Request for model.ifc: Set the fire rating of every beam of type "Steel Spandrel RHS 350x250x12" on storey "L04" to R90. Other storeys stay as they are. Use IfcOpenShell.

First a look at what the model holds.

```python
import ifcopenshell
import ifcopenshell.util.element

model = ifcopenshell.open("model.ifc")
print(model.schema)
storey = next(s for s in model.by_type("IfcBuildingStorey") if s.Name == "L04")
beams = [e for e in ifcopenshell.util.element.get_decomposition(storey) if e.is_a("IfcBeam")]
seen = {}
for e in beams:
    element_type = ifcopenshell.util.element.get_type(e)
    key = (element_type.Name if element_type != e and element_type else None, ifcopenshell.util.element.get_pset(e, "Pset_BeamCommon", "FireRating"))
    seen[key] = seen.get(key, 0) + 1
for (name, value), count in sorted(seen.items(), key=str):
    print(count, "x", name, "|", value)
```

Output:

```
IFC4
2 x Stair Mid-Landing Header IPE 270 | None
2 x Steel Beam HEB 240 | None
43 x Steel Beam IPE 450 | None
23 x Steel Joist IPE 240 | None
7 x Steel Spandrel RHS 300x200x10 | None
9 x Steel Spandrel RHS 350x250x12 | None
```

```python
import ifcopenshell
import ifcopenshell.api.pset
import ifcopenshell.util.element

model = ifcopenshell.open("model.ifc")

storey = next(s for s in model.by_type("IfcBuildingStorey") if s.Name == "L04")
beams = [e for e in ifcopenshell.util.element.get_decomposition(storey) if e.is_a("IfcBeam")]

count = 0
for e in beams:
    element_type = ifcopenshell.util.element.get_type(e)
    if element_type in (None, e) or element_type.Name != "Steel Spandrel RHS 350x250x12":
        continue
    # add_pset returns the element's existing set when there is one.
    pset = ifcopenshell.api.pset.add_pset(model, product=e, name="Pset_BeamCommon")
    ifcopenshell.api.pset.edit_pset(model, pset=pset, properties={"FireRating": "R90"})
    count += 1

print(count, "beams updated")

model.write("model_v2.ifc")
```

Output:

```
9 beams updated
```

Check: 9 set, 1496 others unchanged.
